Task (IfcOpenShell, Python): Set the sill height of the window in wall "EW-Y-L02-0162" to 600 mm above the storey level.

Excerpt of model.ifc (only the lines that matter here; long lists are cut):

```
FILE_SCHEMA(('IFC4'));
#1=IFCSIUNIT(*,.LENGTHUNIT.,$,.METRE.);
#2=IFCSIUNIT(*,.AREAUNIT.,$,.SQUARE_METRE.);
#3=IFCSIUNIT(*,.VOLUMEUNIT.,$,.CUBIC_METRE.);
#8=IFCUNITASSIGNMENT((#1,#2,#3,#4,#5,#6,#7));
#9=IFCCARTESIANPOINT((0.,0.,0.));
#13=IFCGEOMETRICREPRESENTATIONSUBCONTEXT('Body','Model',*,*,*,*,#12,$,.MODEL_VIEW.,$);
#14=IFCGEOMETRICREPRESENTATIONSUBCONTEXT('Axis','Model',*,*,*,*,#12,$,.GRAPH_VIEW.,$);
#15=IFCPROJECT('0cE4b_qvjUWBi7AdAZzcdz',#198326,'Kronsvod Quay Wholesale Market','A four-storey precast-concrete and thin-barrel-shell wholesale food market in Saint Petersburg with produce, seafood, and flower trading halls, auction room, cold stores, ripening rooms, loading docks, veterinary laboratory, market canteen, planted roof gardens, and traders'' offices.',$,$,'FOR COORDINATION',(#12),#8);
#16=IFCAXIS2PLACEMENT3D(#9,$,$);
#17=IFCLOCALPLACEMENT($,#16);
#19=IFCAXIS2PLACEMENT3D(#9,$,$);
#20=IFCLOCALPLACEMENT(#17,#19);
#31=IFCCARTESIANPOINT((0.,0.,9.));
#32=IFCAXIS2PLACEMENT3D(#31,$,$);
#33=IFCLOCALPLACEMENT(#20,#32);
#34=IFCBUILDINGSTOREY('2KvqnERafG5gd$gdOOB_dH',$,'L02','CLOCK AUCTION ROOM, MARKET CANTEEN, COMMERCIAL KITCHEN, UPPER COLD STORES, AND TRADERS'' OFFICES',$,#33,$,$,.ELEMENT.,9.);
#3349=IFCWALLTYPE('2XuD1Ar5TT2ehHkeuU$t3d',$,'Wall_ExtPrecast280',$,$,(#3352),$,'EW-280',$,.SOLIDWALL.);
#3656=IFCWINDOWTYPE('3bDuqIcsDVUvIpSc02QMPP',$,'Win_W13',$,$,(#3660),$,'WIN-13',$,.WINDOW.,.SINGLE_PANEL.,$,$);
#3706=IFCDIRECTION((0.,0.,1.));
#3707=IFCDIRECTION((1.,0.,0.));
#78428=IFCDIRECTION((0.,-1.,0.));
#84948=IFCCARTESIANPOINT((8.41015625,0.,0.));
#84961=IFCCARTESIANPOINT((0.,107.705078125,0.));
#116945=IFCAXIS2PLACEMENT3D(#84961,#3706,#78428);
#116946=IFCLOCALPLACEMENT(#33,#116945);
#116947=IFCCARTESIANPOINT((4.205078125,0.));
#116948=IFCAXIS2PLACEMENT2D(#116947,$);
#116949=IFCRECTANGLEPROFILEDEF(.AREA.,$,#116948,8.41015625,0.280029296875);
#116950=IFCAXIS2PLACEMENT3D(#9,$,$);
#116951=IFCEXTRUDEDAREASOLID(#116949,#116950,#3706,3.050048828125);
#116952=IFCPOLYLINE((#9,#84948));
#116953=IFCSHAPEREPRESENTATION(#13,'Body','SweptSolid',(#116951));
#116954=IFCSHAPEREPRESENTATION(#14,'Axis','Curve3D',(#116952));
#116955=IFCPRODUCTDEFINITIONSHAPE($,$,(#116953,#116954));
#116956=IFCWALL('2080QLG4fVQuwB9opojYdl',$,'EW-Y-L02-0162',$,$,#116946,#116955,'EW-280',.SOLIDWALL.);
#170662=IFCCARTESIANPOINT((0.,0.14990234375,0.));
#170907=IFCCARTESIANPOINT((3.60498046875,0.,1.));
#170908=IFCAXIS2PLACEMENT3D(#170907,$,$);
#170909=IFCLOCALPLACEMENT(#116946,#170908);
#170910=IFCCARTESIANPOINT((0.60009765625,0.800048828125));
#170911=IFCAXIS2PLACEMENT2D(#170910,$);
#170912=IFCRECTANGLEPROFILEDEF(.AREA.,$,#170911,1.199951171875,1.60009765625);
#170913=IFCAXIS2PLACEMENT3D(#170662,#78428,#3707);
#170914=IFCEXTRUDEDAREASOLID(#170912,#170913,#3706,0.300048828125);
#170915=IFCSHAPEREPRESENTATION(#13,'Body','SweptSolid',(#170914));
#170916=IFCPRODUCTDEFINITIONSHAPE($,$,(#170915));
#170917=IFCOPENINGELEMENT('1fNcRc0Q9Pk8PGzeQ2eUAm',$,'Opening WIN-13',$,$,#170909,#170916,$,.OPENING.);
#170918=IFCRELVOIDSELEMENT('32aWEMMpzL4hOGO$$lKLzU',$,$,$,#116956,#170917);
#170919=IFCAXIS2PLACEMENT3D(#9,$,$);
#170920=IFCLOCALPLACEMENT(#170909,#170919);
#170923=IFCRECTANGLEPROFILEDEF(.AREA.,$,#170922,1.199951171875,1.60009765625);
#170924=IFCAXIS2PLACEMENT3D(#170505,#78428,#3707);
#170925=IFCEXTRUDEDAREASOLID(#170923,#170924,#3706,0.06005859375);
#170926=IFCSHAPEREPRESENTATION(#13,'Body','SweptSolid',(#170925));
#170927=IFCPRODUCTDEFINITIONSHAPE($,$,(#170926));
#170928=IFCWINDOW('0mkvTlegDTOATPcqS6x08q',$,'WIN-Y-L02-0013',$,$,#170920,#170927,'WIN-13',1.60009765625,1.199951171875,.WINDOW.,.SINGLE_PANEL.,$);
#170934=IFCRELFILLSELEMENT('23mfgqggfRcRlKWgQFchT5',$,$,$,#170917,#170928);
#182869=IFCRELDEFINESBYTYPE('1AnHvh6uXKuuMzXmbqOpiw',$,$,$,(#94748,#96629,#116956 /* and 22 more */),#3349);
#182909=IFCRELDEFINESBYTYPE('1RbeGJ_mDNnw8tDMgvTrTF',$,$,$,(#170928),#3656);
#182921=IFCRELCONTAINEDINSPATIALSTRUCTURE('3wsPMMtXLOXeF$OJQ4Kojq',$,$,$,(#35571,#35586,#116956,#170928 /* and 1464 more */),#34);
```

```python
import numpy as np
import ifcopenshell
import ifcopenshell.api.geometry
import ifcopenshell.geom
import ifcopenshell.util.element
import ifcopenshell.util.placement
import ifcopenshell.util.shape
import ifcopenshell.util.unit

model = ifcopenshell.open("model.ifc")
unit_scale = ifcopenshell.util.unit.calculate_unit_scale(model)

window = model.by_id(170928)
opening = window.FillsVoids[0].RelatingOpeningElement
storey = ifcopenshell.util.element.get_container(window, ifc_class="IfcBuildingStorey")
level = ifcopenshell.util.placement.get_local_placement(storey.ObjectPlacement)[2, 3]

# The opening's origin need not be at the sill, so measure its lowest point.
shape = ifcopenshell.geom.create_shape(ifcopenshell.geom.settings(), opening)
bottom = ifcopenshell.util.shape.get_shape_bottom_elevation(shape, shape.geometry) / unit_scale
dz = level + 0.6 / unit_scale - bottom

shift = np.array([0.0, 0.0, dz])
# The window is placed relative to its opening, so it follows when the opening moves.
matrix = ifcopenshell.util.placement.get_local_placement(opening.ObjectPlacement)
matrix[:3, 3] += shift
ifcopenshell.api.geometry.edit_object_placement(
    model, product=opening, matrix=matrix, is_si=False, should_transform_children=True
)

print(f"moved by {dz * unit_scale:+.3f} m")

model.write("model-out.ifc")
```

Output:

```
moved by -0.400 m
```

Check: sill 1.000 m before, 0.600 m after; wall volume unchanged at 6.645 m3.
